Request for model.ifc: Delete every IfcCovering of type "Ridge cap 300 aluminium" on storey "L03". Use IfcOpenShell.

First a look at what the model holds.

```python
import ifcopenshell
import ifcopenshell.util.element

model = ifcopenshell.open("model.ifc")
print(model.schema)
storey = next(s for s in model.by_type("IfcBuildingStorey") if s.Name == "L03")
coverings = [e for e in ifcopenshell.util.element.get_decomposition(storey) if e.is_a("IfcCovering")]
seen = {}
for e in coverings:
    element_type = ifcopenshell.util.element.get_type(e)
    name = element_type.Name if element_type not in (None, e) else None
    seen[name] = seen.get(name, 0) + 1
for name, count in sorted(seen.items(), key=str):
    print(count, "x", name)
```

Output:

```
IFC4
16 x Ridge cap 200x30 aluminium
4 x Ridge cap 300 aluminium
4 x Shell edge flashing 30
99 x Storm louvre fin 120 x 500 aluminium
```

```python
import ifcopenshell
import ifcopenshell.api.root
import ifcopenshell.util.element

model = ifcopenshell.open("model.ifc")

storey = next(s for s in model.by_type("IfcBuildingStorey") if s.Name == "L03")
coverings = [e for e in ifcopenshell.util.element.get_decomposition(storey) if e.is_a("IfcCovering")]
targets = [e for e in coverings if (t := ifcopenshell.util.element.get_type(e)) not in (None, e) and t.Name == "Ridge cap 300 aluminium"]

for e in targets:
    ifcopenshell.api.root.remove_product(model, product=e)
print(len(targets), "removed")

model.write("model_edited.ifc")
```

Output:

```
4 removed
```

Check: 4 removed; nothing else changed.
